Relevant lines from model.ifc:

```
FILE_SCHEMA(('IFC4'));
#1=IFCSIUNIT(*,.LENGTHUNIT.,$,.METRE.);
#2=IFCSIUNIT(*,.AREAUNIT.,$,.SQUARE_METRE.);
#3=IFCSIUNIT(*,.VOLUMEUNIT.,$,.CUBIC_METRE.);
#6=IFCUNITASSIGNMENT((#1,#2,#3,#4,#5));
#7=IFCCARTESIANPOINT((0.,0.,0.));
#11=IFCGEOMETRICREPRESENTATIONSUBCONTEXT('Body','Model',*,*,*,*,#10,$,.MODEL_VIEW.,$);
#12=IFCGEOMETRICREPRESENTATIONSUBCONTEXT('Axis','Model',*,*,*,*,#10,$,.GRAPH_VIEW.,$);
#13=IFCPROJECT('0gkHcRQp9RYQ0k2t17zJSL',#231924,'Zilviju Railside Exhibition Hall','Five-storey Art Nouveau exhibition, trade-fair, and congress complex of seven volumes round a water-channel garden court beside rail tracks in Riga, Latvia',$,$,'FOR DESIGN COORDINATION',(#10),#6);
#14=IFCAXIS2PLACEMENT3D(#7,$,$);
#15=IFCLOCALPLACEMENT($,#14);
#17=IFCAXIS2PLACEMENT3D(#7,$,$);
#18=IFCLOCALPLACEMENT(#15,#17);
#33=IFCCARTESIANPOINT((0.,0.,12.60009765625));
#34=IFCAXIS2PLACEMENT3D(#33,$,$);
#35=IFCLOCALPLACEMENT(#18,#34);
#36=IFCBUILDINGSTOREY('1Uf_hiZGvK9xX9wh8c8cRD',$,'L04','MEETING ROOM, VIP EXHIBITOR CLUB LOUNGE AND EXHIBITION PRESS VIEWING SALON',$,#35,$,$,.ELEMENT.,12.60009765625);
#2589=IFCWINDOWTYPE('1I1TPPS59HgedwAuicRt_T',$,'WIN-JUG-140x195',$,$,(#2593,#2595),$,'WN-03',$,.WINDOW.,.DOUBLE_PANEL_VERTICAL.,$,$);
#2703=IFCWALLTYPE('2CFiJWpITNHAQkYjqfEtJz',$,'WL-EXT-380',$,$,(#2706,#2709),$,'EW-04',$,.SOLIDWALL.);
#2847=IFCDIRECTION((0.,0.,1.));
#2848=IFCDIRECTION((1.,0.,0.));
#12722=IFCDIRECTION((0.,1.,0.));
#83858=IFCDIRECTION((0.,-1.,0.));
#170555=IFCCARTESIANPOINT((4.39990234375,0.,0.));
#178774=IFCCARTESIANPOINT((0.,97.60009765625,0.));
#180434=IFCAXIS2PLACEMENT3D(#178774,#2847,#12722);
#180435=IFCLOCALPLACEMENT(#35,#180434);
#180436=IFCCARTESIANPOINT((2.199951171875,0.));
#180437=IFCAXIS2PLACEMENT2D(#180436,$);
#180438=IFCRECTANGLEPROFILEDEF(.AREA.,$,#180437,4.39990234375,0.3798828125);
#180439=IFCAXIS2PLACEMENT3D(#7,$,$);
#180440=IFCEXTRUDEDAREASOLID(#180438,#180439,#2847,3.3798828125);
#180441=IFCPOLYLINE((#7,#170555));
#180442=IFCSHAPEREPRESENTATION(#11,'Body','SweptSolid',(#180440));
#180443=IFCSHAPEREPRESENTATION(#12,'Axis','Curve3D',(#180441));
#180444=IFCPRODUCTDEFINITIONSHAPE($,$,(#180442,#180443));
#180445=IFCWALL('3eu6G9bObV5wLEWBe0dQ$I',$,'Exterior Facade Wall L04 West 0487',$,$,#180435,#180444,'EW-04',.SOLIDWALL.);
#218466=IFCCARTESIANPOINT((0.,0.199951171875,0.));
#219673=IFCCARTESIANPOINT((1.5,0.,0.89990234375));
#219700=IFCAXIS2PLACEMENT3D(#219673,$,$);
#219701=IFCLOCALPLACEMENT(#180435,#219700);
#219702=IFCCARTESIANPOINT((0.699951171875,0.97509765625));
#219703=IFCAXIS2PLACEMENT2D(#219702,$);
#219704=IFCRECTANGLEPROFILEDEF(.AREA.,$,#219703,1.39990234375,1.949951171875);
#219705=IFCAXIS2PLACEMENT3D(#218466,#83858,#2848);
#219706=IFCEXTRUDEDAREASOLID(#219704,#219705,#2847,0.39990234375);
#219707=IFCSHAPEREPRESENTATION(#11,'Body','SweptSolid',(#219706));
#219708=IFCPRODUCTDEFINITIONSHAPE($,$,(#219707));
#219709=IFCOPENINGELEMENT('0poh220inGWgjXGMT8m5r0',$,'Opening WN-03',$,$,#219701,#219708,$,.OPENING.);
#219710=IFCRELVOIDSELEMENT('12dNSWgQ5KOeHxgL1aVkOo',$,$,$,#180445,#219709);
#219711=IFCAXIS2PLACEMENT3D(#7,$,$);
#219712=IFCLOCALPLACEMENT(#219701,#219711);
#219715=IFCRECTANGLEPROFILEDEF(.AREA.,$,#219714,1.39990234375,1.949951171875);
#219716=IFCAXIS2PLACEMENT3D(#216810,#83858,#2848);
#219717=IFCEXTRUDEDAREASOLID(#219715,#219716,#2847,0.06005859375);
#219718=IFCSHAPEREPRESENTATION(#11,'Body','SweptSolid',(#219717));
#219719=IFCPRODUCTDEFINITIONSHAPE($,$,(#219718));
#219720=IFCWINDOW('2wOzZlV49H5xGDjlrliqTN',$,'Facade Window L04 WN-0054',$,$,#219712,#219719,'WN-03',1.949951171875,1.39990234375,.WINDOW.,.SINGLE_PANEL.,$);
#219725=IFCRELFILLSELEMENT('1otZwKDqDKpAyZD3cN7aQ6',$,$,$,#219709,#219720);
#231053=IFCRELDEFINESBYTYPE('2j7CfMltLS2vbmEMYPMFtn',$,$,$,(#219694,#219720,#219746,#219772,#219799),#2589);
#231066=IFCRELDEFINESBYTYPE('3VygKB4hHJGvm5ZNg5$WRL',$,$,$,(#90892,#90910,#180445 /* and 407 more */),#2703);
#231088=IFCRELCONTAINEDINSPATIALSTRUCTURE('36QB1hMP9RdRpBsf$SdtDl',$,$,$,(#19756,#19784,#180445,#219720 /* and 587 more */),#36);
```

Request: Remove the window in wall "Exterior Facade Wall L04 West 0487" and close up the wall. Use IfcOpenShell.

```python
import ifcopenshell
import ifcopenshell.api.feature
import ifcopenshell.api.root
import ifcopenshell.geom
import ifcopenshell.util.shape

model = ifcopenshell.open("model.ifc")
settings = ifcopenshell.geom.settings()


def volume(element):
    """Net volume in cubic metres, openings subtracted."""
    shape = ifcopenshell.geom.create_shape(settings, element)
    return ifcopenshell.util.shape.get_volume(shape.geometry)


window = model.by_guid("2wOzZlV49H5xGDjlrliqTN")
opening = window.FillsVoids[0].RelatingOpeningElement
wall = opening.VoidsElements[0].RelatingBuildingElement
before = volume(wall)

ifcopenshell.api.root.remove_product(model, product=window)
ifcopenshell.api.feature.remove_feature(model, feature=opening)

after = volume(wall)

print(f"wall volume {before:.3f} -> {after:.3f} m3")

model.write("model-out.ifc")
```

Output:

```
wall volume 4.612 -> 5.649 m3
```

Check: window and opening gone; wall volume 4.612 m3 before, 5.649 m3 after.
